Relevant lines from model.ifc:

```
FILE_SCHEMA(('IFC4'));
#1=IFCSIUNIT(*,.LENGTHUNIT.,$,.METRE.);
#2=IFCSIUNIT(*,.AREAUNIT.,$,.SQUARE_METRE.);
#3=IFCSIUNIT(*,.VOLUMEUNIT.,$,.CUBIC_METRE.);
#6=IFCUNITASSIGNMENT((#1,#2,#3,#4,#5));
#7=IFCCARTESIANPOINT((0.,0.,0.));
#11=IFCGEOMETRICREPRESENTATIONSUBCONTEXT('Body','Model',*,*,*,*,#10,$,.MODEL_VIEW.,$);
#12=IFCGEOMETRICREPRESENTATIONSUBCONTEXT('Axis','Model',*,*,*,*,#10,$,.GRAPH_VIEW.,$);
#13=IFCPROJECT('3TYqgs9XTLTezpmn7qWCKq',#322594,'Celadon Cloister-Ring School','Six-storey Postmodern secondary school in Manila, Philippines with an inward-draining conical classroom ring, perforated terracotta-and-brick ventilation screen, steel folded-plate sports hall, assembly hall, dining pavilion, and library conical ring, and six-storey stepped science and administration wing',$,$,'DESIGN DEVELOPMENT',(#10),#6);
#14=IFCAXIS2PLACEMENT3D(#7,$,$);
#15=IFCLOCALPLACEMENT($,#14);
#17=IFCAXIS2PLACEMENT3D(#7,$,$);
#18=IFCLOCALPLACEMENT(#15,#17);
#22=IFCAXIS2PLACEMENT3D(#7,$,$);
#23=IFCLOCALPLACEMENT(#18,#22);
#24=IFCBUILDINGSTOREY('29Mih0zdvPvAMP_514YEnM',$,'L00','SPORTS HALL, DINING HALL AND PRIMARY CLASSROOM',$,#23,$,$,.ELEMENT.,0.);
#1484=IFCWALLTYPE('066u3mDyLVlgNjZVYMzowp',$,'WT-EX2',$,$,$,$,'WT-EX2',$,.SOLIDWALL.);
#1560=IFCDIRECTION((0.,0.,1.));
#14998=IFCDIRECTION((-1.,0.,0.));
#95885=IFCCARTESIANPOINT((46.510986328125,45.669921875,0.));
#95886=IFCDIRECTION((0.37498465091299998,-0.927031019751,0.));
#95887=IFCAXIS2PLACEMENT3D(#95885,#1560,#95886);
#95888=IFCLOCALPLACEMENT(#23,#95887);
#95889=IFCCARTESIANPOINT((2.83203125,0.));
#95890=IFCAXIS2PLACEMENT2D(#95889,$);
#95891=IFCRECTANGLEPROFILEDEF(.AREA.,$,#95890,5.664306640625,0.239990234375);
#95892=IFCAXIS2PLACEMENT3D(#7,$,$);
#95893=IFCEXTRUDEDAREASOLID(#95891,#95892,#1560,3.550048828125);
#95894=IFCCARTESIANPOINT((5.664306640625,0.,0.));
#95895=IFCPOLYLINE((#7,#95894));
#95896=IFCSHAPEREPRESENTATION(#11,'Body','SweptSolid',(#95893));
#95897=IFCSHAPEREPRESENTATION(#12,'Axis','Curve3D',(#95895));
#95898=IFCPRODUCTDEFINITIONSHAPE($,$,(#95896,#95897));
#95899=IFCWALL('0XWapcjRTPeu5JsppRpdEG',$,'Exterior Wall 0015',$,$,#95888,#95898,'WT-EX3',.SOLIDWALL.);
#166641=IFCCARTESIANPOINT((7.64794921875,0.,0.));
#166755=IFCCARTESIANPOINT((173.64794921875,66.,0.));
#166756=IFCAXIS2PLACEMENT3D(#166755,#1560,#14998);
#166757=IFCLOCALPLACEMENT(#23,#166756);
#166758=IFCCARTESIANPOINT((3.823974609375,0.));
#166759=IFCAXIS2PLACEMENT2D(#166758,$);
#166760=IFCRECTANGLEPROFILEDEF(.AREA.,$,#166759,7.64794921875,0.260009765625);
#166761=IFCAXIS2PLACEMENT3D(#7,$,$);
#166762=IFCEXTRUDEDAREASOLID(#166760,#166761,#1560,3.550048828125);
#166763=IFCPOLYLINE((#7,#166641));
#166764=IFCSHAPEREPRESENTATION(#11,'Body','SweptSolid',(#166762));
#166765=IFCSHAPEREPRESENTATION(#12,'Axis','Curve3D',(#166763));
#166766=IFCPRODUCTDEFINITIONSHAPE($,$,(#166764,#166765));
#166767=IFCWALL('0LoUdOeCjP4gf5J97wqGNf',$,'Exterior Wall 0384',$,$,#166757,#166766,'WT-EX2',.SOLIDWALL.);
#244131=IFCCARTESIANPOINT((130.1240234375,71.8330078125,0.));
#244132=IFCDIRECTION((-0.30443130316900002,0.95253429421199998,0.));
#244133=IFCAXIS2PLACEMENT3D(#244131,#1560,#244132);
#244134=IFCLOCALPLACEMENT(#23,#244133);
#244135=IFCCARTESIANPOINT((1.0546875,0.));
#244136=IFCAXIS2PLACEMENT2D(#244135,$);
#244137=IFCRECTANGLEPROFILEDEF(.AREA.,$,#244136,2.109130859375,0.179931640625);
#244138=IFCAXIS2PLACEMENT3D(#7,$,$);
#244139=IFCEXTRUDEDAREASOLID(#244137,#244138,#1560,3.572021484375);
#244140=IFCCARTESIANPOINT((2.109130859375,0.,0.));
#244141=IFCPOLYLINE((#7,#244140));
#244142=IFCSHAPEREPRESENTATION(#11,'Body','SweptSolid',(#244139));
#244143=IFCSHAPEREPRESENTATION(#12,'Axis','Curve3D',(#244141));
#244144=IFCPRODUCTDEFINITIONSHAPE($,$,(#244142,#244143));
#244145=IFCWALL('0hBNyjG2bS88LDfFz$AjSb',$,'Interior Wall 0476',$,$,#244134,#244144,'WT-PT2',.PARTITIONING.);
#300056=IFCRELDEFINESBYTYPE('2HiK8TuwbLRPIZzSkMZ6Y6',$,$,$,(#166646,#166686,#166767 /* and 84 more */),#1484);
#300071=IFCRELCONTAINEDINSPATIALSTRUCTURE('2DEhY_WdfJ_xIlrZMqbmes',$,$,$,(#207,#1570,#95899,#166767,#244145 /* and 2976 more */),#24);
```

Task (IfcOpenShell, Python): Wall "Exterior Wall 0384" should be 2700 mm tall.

```python
import ifcopenshell
import ifcopenshell.geom
import ifcopenshell.util.representation
import ifcopenshell.util.shape
import ifcopenshell.util.unit

model = ifcopenshell.open("model.ifc")
unit_scale = ifcopenshell.util.unit.calculate_unit_scale(model)
settings = ifcopenshell.geom.settings()


def volume(element):
    """Net volume in cubic metres, openings subtracted."""
    shape = ifcopenshell.geom.create_shape(settings, element)
    return ifcopenshell.util.shape.get_volume(shape.geometry)


wall = model.by_guid("0LoUdOeCjP4gf5J97wqGNf")
before = volume(wall)

body = ifcopenshell.util.representation.get_representation(wall, "Model", "Body")
solid = body.Items[0]
old_height = solid.Depth
solid.Depth = 2.7 / unit_scale
after = volume(wall)

print(f"height {old_height:g} -> {solid.Depth:g}, volume {before:.3f} -> {after:.3f} m3")

model.write("model_edited.ifc")
```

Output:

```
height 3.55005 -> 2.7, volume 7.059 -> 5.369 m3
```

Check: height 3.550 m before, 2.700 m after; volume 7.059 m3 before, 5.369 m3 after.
